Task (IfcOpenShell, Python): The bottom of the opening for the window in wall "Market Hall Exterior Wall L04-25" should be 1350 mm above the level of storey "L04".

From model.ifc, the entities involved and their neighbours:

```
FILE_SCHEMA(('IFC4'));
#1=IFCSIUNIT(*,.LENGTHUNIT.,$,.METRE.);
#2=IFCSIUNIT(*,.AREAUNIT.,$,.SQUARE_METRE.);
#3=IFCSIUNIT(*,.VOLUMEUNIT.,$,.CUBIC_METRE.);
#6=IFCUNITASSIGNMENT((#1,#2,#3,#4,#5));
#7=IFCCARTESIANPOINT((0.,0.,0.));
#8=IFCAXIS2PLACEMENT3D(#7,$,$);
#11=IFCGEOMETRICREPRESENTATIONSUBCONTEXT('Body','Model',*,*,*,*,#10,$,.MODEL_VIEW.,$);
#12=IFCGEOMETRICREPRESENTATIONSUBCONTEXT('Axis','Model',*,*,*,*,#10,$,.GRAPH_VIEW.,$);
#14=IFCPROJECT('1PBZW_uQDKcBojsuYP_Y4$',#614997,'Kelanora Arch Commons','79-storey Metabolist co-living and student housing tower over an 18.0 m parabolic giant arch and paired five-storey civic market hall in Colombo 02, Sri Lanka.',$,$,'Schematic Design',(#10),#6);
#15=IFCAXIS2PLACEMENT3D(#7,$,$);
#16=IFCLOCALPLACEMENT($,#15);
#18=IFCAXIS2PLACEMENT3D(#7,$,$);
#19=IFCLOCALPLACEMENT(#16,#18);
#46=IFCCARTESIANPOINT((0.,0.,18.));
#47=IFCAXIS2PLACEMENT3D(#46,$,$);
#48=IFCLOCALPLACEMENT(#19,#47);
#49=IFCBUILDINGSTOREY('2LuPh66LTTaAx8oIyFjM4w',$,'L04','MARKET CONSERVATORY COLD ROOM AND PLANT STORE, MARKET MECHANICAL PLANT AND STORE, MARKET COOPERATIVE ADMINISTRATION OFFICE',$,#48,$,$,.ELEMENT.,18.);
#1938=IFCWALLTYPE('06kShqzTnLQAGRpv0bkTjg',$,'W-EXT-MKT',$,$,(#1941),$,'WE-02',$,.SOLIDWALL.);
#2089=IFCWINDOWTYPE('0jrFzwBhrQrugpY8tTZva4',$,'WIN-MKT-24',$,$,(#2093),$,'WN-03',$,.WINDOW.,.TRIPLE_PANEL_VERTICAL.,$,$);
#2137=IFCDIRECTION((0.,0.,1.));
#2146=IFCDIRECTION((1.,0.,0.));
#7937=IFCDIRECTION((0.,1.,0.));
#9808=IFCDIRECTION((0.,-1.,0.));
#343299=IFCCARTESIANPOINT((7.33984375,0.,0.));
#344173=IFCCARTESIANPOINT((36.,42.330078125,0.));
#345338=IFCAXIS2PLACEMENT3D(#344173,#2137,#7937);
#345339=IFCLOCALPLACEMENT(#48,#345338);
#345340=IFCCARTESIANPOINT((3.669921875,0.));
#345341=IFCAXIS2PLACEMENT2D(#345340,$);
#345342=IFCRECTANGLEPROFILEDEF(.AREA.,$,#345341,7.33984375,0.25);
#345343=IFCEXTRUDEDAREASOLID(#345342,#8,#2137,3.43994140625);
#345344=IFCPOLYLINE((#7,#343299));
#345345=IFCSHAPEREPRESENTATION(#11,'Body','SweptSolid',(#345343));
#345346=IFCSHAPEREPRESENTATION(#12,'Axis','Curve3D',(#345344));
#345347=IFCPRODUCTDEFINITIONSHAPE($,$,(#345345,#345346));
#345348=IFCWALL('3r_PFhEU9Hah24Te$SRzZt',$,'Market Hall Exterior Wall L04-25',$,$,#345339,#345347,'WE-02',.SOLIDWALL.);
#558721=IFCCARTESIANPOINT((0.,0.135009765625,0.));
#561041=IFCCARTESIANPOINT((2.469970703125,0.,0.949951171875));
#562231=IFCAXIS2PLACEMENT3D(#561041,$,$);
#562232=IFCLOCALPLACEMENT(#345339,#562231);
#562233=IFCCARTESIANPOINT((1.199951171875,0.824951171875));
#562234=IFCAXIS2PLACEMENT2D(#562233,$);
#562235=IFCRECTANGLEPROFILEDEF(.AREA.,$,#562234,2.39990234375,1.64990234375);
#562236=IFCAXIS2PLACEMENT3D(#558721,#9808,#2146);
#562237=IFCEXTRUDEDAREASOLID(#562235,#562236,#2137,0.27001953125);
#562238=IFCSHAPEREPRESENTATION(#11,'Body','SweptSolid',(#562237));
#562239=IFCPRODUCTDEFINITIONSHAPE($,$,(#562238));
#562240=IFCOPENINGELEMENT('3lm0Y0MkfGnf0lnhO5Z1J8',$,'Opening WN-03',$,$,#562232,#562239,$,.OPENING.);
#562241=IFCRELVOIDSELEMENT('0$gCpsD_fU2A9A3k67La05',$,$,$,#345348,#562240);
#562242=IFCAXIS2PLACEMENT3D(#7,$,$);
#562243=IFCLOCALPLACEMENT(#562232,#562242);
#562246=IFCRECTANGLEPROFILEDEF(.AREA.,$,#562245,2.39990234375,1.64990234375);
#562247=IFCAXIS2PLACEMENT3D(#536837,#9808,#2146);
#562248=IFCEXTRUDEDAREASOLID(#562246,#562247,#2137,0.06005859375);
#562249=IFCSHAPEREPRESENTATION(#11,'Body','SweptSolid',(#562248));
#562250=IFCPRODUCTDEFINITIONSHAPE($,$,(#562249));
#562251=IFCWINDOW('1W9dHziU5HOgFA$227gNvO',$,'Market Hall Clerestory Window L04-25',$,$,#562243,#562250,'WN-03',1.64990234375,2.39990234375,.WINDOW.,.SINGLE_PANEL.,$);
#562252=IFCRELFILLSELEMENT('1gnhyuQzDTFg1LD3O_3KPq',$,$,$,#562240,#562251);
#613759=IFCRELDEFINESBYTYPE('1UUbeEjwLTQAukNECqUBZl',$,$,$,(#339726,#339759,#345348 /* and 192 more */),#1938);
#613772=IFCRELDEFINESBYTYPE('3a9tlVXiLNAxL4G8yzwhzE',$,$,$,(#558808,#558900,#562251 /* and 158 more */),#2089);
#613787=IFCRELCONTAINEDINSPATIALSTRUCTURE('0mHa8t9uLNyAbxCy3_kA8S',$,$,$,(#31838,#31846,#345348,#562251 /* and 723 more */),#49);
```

```python
import numpy as np
import ifcopenshell
import ifcopenshell.api.geometry
import ifcopenshell.geom
import ifcopenshell.util.element
import ifcopenshell.util.placement
import ifcopenshell.util.shape
import ifcopenshell.util.unit

model = ifcopenshell.open("model.ifc")
unit_scale = ifcopenshell.util.unit.calculate_unit_scale(model)

window = model.by_id(562251)
opening = window.FillsVoids[0].RelatingOpeningElement
storey = ifcopenshell.util.element.get_container(window, ifc_class="IfcBuildingStorey")
level = ifcopenshell.util.placement.get_local_placement(storey.ObjectPlacement)[2, 3]

# The opening's origin need not be at the sill, so measure its lowest point.
shape = ifcopenshell.geom.create_shape(ifcopenshell.geom.settings(), opening)
bottom = ifcopenshell.util.shape.get_shape_bottom_elevation(shape, shape.geometry) / unit_scale
dz = level + 1.35 / unit_scale - bottom

shift = np.array([0.0, 0.0, dz])
# The window is placed relative to its opening, so it follows when the opening moves.
matrix = ifcopenshell.util.placement.get_local_placement(opening.ObjectPlacement)
matrix[:3, 3] += shift
ifcopenshell.api.geometry.edit_object_placement(
    model, product=opening, matrix=matrix, is_si=False, should_transform_children=True
)

print(f"moved by {dz * unit_scale:+.3f} m")

model.write("model_v2.ifc")
```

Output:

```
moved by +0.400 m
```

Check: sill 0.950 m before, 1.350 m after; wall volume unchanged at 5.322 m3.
